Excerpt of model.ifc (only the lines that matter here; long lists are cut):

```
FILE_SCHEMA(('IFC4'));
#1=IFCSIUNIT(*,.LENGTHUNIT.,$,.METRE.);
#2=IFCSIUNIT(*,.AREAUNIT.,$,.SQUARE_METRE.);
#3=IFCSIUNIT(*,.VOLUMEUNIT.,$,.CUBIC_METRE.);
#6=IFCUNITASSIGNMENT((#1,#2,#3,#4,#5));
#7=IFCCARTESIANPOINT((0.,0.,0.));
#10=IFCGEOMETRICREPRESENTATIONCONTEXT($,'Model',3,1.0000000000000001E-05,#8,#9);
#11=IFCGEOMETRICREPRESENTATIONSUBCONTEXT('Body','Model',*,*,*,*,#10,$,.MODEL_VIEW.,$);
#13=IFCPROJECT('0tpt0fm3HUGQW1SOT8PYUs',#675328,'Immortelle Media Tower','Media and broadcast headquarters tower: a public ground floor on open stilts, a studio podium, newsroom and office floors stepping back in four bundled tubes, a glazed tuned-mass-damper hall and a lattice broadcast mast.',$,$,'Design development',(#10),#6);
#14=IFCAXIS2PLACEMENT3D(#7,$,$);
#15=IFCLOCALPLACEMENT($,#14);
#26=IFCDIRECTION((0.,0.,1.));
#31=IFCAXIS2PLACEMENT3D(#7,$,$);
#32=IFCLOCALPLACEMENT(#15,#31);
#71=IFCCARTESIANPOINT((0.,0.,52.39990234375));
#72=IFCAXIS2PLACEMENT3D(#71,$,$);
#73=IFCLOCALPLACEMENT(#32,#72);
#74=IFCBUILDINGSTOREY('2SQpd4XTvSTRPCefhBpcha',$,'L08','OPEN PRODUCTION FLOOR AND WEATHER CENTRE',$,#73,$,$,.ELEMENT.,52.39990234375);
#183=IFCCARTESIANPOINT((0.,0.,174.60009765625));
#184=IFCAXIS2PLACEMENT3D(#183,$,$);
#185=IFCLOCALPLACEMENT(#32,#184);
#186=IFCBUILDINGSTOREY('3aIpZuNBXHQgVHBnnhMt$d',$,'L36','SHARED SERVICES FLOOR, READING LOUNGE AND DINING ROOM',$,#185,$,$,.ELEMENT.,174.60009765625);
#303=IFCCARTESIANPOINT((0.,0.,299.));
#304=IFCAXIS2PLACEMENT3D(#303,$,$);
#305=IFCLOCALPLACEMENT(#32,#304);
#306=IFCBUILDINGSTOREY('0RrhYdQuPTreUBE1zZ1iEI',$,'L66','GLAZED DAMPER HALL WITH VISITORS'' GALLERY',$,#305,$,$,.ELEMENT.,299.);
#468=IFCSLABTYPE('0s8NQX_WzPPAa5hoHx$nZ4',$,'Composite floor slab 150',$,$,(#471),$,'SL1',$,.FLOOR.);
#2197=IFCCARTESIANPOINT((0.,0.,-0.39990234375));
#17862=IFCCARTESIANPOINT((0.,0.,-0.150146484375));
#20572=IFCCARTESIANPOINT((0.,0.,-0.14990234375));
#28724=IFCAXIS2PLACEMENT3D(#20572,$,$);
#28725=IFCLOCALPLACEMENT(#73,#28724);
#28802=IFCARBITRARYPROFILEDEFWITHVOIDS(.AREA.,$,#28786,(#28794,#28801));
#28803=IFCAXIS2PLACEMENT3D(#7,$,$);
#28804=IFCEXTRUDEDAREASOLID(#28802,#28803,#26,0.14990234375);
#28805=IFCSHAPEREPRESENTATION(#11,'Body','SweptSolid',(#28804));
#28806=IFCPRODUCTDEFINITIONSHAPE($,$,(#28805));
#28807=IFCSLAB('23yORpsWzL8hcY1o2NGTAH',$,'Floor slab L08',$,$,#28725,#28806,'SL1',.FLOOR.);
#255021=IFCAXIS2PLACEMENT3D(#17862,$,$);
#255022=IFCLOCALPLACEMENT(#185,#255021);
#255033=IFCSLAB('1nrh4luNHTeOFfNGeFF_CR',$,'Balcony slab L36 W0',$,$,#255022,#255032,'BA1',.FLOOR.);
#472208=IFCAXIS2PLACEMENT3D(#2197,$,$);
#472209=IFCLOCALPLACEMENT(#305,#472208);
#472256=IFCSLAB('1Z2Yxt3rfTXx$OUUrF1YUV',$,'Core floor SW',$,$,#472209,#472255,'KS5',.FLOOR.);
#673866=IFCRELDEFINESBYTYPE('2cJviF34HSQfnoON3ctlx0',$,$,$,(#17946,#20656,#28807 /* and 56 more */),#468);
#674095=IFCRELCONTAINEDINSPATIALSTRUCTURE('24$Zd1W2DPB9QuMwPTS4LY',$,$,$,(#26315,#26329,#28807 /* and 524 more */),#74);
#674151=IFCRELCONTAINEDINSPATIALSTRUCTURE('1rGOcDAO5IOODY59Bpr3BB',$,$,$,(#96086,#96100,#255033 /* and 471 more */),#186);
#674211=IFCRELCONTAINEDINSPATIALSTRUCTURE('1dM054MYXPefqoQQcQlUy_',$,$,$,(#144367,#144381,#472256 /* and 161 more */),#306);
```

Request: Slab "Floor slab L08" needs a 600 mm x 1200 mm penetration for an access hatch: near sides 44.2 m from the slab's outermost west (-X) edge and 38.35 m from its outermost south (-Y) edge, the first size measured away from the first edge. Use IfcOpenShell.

```python
import numpy as np
import ifcopenshell
import ifcopenshell.api.feature
import ifcopenshell.api.geometry
import ifcopenshell.api.root
import ifcopenshell.geom
import ifcopenshell.util.placement
import ifcopenshell.util.representation
import ifcopenshell.util.shape
import ifcopenshell.util.unit

model = ifcopenshell.open("model.ifc")
unit_scale = ifcopenshell.util.unit.calculate_unit_scale(model)
settings = ifcopenshell.geom.settings()


def volume(element):
    """Net volume in cubic metres, openings subtracted."""
    shape = ifcopenshell.geom.create_shape(settings, element)
    return ifcopenshell.util.shape.get_volume(shape.geometry)


slab = model.by_guid("23yORpsWzL8hcY1o2NGTAH")
before = volume(slab)

# Extent in the slab's own axes, in metres. The edges named are its -X and -Y sides.
slab_shape = ifcopenshell.geom.create_shape(settings, slab)
vertices = ifcopenshell.util.shape.get_vertices(slab_shape.geometry)
x_min, y_min, bottom = vertices.min(axis=0)
top = vertices[:, 2].max()

opening = ifcopenshell.api.root.create_entity(model, ifc_class="IfcOpeningElement", name="Access hatch opening", predefined_type="OPENING")
context = ifcopenshell.util.representation.get_context(model, "Model", "Body", "MODEL_VIEW")
width, depth = 0.6, 1.2
outline = [(0.0, 0.0), (width, 0.0), (width, depth), (0.0, depth), (0.0, 0.0)]
# Overshoot both faces by 50 mm so the cut is clean.
shape = ifcopenshell.api.geometry.add_slab_representation(
    model, context=context, depth=top - bottom + 0.1, polyline=outline
)
ifcopenshell.api.geometry.assign_representation(model, product=opening, representation=shape)

matrix = ifcopenshell.util.placement.get_local_placement(slab.ObjectPlacement)
matrix[:, 3] = matrix @ np.append(np.array([x_min + 44.2, y_min + 38.35, bottom - 0.05]) / unit_scale, 1.0)
ifcopenshell.api.geometry.edit_object_placement(model, product=opening, matrix=matrix, is_si=False)
ifcopenshell.api.feature.add_feature(model, feature=opening, element=slab)

after = volume(slab)

print(f"slab volume {before:.3f} -> {after:.3f} m3")

model.write("model-out.ifc")
```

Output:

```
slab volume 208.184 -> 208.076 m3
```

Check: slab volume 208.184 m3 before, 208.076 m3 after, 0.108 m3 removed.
